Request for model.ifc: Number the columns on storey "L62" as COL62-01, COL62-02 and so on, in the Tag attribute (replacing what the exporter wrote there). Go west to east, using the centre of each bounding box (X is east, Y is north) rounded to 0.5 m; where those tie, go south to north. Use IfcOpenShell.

First a look at what the model holds.

```python
import ifcopenshell
import ifcopenshell.util.element
import ifcopenshell.util.placement

model = ifcopenshell.open("model.ifc")
print(model.schema)
storey = next(s for s in model.by_type("IfcBuildingStorey") if s.Name == "L62")
columns = [e for e in ifcopenshell.util.element.get_decomposition(storey) if e.is_a("IfcColumn")]
for e in sorted(columns, key=lambda e: e.id()):
    origin = ifcopenshell.util.placement.get_local_placement(e.ObjectPlacement)[:3, 3]
    print(e.id(), e.Tag, e.Name, origin.round(2) + 0.0, sep=" | ")
```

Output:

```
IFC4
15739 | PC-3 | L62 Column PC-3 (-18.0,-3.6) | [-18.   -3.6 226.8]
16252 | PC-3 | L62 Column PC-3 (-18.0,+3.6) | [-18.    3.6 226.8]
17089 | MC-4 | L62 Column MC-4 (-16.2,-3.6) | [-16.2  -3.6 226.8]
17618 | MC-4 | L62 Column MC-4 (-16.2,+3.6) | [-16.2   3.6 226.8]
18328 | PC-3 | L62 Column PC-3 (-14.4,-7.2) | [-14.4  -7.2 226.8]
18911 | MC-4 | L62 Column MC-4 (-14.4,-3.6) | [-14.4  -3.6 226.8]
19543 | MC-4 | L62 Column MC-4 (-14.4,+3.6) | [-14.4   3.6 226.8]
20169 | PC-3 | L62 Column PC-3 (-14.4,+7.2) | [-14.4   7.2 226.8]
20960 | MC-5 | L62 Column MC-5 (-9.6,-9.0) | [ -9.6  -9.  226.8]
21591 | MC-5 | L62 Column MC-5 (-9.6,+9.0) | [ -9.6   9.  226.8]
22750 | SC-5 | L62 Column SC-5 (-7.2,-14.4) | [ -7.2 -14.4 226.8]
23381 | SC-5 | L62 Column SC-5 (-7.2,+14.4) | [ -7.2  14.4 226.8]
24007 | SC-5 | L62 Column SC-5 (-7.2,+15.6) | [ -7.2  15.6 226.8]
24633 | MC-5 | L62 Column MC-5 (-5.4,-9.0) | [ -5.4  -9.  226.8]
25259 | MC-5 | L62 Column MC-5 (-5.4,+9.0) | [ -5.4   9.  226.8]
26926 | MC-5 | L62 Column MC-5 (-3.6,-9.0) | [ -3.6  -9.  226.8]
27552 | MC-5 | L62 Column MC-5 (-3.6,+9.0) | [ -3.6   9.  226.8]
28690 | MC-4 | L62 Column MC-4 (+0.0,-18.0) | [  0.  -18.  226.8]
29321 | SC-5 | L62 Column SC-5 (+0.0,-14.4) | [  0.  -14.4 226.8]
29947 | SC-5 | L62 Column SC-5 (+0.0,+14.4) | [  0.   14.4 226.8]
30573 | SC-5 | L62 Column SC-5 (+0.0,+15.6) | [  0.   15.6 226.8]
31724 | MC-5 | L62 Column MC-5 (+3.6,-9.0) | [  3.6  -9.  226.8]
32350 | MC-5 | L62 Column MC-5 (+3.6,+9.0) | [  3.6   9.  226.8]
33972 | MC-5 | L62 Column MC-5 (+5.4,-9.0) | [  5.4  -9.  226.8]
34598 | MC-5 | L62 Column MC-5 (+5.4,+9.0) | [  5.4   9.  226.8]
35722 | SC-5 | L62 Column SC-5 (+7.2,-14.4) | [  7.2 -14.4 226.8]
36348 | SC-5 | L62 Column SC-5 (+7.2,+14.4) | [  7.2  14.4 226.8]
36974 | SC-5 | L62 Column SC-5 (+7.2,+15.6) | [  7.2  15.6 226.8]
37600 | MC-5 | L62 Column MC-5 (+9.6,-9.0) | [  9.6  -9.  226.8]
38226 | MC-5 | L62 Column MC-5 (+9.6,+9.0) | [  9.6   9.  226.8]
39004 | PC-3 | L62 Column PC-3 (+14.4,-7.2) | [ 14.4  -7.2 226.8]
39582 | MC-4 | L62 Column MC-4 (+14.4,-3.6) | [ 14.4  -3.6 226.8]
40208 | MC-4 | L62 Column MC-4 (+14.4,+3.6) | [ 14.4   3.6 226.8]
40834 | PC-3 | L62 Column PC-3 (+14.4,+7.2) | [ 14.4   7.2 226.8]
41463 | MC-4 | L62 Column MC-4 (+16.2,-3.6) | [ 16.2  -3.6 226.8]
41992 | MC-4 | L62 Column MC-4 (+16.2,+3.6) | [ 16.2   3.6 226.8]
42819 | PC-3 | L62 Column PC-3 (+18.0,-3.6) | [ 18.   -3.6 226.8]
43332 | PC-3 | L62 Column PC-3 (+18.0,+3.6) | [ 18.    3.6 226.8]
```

```python
import ifcopenshell
import ifcopenshell.geom
import ifcopenshell.util.element
import ifcopenshell.util.shape

model = ifcopenshell.open("model.ifc")
settings = ifcopenshell.geom.settings()
settings.set("use-world-coords", True)


def centre(element):
    shape = ifcopenshell.geom.create_shape(settings, element)
    return ifcopenshell.util.shape.get_bbox_centroid(shape.geometry)


storey = next(s for s in model.by_type("IfcBuildingStorey") if s.Name == "L62")
columns = [e for e in ifcopenshell.util.element.get_decomposition(storey) if e.is_a("IfcColumn")]

# Insertion points can sit at a corner or the storey origin, so sort by the geometry (in metres).
centres = {e: centre(e) for e in columns}
columns.sort(key=lambda e: (round(centres[e][0] / 0.5), centres[e][1]))

for i, e in enumerate(columns, start=1):
    number = f"COL62-{i:02d}"
    e.Tag = number
    print(e.id(), number)

model.write("model_v2.ifc")
```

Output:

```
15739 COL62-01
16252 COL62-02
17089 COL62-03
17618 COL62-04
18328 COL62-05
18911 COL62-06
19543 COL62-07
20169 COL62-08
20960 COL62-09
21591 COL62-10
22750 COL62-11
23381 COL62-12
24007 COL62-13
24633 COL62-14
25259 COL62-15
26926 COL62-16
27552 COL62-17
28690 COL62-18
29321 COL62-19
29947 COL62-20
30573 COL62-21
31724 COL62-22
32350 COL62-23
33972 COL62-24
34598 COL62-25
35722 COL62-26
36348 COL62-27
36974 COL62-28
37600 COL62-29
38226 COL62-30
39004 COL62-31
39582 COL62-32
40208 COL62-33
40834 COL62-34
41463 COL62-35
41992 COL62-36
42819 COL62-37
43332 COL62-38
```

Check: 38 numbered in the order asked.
